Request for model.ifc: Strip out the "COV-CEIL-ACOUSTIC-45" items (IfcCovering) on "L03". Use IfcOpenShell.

First a look at what the model holds.

```python
import ifcopenshell
import ifcopenshell.util.element

model = ifcopenshell.open("model.ifc")
print(model.schema)
storey = next(s for s in model.by_type("IfcBuildingStorey") if s.Name == "L03")
coverings = [e for e in ifcopenshell.util.element.get_decomposition(storey) if e.is_a("IfcCovering")]
seen = {}
for e in coverings:
    element_type = ifcopenshell.util.element.get_type(e)
    name = element_type.Name if element_type not in (None, e) else None
    seen[name] = seen.get(name, 0) + 1
for name, count in sorted(seen.items(), key=str):
    print(count, "x", name)
```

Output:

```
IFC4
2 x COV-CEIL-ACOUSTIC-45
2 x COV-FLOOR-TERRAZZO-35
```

```python
import ifcopenshell
import ifcopenshell.api.root
import ifcopenshell.util.element

model = ifcopenshell.open("model.ifc")

storey = next(s for s in model.by_type("IfcBuildingStorey") if s.Name == "L03")
coverings = [e for e in ifcopenshell.util.element.get_decomposition(storey) if e.is_a("IfcCovering")]
targets = [e for e in coverings if (t := ifcopenshell.util.element.get_type(e)) not in (None, e) and t.Name == "COV-CEIL-ACOUSTIC-45"]

for e in targets:
    ifcopenshell.api.root.remove_product(model, product=e)
print(len(targets), "removed")

model.write("model_v2.ifc")
```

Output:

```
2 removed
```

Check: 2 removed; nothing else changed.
